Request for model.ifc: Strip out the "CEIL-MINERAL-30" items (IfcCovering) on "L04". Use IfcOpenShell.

First a look at what the model holds.

```python
import ifcopenshell
import ifcopenshell.util.element

model = ifcopenshell.open("model.ifc")
print(model.schema)
storey = next(s for s in model.by_type("IfcBuildingStorey") if s.Name == "L04")
coverings = [e for e in ifcopenshell.util.element.get_decomposition(storey) if e.is_a("IfcCovering")]
seen = {}
for e in coverings:
    element_type = ifcopenshell.util.element.get_type(e)
    name = element_type.Name if element_type not in (None, e) else None
    seen[name] = seen.get(name, 0) + 1
for name, count in sorted(seen.items(), key=str):
    print(count, "x", name)
```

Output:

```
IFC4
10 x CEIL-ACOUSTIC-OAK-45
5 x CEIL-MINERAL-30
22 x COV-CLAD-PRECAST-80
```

```python
import ifcopenshell
import ifcopenshell.api.root
import ifcopenshell.util.element

model = ifcopenshell.open("model.ifc")

storey = next(s for s in model.by_type("IfcBuildingStorey") if s.Name == "L04")
coverings = [e for e in ifcopenshell.util.element.get_decomposition(storey) if e.is_a("IfcCovering")]
targets = [e for e in coverings if (t := ifcopenshell.util.element.get_type(e)) not in (None, e) and t.Name == "CEIL-MINERAL-30"]

for e in targets:
    ifcopenshell.api.root.remove_product(model, product=e)
print(len(targets), "removed")

model.write("model_v2.ifc")
```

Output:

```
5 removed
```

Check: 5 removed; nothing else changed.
